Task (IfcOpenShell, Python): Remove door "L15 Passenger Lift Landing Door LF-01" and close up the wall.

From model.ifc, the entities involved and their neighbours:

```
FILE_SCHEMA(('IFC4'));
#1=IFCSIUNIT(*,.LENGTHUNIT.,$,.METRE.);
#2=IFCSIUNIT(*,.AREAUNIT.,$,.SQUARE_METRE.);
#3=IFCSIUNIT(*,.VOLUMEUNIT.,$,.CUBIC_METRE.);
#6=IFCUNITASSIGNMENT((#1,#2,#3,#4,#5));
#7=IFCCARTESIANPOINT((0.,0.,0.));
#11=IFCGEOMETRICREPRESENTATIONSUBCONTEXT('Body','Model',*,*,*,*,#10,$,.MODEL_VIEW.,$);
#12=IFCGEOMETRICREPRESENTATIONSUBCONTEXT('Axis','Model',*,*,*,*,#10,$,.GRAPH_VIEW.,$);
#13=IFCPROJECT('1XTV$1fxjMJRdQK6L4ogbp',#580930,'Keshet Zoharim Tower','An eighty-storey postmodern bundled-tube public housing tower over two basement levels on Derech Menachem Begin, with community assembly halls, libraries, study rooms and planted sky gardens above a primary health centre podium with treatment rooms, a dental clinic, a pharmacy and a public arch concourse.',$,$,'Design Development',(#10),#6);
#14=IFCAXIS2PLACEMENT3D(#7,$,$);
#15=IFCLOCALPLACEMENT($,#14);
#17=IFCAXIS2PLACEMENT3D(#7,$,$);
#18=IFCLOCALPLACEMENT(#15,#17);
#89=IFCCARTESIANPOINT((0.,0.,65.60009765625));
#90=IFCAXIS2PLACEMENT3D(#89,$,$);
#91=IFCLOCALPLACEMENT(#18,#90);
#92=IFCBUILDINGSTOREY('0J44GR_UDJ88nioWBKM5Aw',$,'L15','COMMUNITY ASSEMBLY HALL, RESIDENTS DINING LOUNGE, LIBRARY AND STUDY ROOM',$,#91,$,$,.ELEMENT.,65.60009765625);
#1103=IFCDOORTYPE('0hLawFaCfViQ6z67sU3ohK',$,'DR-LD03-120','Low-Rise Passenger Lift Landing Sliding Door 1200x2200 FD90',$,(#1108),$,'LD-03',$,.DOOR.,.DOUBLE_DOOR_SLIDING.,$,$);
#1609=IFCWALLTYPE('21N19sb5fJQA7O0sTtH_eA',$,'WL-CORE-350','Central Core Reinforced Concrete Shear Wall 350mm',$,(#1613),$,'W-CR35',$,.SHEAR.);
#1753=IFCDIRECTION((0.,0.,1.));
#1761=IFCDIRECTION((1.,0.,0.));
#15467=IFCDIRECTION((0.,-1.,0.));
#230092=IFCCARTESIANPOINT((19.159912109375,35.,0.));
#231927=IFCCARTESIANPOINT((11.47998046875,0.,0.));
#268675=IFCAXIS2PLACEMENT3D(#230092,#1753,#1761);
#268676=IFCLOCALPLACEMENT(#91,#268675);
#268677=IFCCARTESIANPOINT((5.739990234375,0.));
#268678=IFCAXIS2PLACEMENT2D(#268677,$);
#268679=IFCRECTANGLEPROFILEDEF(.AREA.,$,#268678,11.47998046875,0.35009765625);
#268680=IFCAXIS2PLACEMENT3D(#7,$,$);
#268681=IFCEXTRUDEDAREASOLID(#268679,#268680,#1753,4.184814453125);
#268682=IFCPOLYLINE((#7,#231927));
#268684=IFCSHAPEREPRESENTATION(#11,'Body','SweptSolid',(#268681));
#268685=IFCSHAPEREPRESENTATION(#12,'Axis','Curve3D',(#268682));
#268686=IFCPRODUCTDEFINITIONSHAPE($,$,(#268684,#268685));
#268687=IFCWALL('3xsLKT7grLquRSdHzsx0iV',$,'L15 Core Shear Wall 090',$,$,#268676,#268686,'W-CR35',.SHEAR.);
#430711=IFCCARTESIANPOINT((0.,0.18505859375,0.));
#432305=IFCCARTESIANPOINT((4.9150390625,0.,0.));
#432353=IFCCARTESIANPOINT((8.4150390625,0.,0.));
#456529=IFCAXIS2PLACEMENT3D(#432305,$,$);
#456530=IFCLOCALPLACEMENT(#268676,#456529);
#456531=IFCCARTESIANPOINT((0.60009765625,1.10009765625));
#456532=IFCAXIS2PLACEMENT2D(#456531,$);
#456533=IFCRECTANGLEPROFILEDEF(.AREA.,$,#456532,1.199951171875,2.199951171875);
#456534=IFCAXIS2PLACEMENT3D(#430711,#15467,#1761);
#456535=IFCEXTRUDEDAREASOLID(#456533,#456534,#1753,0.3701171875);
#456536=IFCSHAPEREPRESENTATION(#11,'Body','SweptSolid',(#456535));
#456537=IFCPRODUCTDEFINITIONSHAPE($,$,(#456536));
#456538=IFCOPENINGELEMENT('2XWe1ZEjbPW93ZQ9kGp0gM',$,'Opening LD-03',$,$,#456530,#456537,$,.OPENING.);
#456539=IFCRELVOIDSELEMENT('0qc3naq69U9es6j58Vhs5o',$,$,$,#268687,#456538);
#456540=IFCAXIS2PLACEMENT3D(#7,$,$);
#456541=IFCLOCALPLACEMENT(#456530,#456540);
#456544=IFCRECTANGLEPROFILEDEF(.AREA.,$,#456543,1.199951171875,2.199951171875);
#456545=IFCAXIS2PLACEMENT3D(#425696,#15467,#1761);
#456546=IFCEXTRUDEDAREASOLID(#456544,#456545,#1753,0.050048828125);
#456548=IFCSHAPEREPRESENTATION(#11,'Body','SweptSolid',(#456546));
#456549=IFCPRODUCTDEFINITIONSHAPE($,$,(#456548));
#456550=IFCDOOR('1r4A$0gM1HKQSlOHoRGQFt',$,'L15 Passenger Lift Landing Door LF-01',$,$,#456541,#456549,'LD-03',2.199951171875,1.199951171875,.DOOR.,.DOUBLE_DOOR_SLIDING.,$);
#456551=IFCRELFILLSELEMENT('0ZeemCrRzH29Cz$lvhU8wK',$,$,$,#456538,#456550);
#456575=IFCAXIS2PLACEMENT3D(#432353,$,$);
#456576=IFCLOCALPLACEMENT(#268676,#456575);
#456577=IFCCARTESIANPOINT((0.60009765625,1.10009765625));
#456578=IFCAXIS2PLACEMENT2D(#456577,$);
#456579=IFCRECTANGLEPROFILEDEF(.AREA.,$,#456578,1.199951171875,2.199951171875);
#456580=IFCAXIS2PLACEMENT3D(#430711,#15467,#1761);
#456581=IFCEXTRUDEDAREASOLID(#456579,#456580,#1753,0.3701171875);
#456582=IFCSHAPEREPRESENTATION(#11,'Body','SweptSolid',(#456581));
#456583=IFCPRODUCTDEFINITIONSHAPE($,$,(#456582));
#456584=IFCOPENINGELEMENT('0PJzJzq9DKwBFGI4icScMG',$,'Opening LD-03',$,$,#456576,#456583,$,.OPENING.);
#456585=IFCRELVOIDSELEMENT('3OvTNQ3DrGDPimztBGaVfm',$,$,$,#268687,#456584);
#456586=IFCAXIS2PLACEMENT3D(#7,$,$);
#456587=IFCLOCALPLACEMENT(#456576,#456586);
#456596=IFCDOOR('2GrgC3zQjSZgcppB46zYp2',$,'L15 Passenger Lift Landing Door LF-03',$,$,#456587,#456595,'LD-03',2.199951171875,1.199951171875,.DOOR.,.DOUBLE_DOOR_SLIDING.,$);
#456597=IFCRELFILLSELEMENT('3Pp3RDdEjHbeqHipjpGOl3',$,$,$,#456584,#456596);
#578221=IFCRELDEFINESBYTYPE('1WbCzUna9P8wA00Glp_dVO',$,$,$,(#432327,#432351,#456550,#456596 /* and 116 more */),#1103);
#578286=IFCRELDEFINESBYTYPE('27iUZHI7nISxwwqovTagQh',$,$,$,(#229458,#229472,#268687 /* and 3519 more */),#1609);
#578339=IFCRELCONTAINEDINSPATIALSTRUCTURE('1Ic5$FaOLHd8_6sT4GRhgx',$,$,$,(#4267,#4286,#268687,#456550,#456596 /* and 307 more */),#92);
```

```python
import ifcopenshell
import ifcopenshell.api.feature
import ifcopenshell.api.root
import ifcopenshell.geom
import ifcopenshell.util.shape

model = ifcopenshell.open("model.ifc")
settings = ifcopenshell.geom.settings()


def volume(element):
    """Net volume in cubic metres, openings subtracted."""
    shape = ifcopenshell.geom.create_shape(settings, element)
    return ifcopenshell.util.shape.get_volume(shape.geometry)


door = model.by_guid("1r4A$0gM1HKQSlOHoRGQFt")
opening = door.FillsVoids[0].RelatingOpeningElement
wall = opening.VoidsElements[0].RelatingBuildingElement
before = volume(wall)

ifcopenshell.api.root.remove_product(model, product=door)
ifcopenshell.api.feature.remove_feature(model, feature=opening)

after = volume(wall)

print(f"wall volume {before:.3f} -> {after:.3f} m3")

model.write("model_v2.ifc")
```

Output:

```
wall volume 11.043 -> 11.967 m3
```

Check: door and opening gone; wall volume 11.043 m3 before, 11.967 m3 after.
